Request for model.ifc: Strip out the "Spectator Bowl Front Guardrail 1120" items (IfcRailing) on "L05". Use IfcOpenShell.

First a look at what the model holds.

```python
import ifcopenshell
import ifcopenshell.util.element

model = ifcopenshell.open("model.ifc")
print(model.schema)
storey = next(s for s in model.by_type("IfcBuildingStorey") if s.Name == "L05")
railings = [e for e in ifcopenshell.util.element.get_decomposition(storey) if e.is_a("IfcRailing")]
seen = {}
for e in railings:
    element_type = ifcopenshell.util.element.get_type(e)
    name = element_type.Name if element_type not in (None, e) else None
    seen[name] = seen.get(name, 0) + 1
for name, count in sorted(seen.items(), key=str):
    print(count, "x", name)
```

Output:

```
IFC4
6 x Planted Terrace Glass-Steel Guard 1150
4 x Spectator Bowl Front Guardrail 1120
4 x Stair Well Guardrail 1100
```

```python
import ifcopenshell
import ifcopenshell.api.root
import ifcopenshell.util.element

model = ifcopenshell.open("model.ifc")

storey = next(s for s in model.by_type("IfcBuildingStorey") if s.Name == "L05")
railings = [e for e in ifcopenshell.util.element.get_decomposition(storey) if e.is_a("IfcRailing")]
targets = [e for e in railings if (t := ifcopenshell.util.element.get_type(e)) not in (None, e) and t.Name == "Spectator Bowl Front Guardrail 1120"]

for e in targets:
    ifcopenshell.api.root.remove_product(model, product=e)
print(len(targets), "removed")

model.write("model_updated.ifc")
```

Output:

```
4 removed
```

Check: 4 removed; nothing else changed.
